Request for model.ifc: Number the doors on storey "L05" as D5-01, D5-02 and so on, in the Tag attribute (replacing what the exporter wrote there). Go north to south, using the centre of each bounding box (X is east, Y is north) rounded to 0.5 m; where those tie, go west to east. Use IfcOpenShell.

First a look at what the model holds.

```python
import ifcopenshell
import ifcopenshell.util.element
import ifcopenshell.util.placement

model = ifcopenshell.open("model.ifc")
print(model.schema)
storey = next(s for s in model.by_type("IfcBuildingStorey") if s.Name == "L05")
doors = [e for e in ifcopenshell.util.element.get_decomposition(storey) if e.is_a("IfcDoor")]
for e in sorted(doors, key=lambda e: e.id()):
    origin = ifcopenshell.util.placement.get_local_placement(e.ObjectPlacement)[:3, 3]
    print(e.id(), e.Tag, e.Name, origin.round(2) + 0.0, sep=" | ")
```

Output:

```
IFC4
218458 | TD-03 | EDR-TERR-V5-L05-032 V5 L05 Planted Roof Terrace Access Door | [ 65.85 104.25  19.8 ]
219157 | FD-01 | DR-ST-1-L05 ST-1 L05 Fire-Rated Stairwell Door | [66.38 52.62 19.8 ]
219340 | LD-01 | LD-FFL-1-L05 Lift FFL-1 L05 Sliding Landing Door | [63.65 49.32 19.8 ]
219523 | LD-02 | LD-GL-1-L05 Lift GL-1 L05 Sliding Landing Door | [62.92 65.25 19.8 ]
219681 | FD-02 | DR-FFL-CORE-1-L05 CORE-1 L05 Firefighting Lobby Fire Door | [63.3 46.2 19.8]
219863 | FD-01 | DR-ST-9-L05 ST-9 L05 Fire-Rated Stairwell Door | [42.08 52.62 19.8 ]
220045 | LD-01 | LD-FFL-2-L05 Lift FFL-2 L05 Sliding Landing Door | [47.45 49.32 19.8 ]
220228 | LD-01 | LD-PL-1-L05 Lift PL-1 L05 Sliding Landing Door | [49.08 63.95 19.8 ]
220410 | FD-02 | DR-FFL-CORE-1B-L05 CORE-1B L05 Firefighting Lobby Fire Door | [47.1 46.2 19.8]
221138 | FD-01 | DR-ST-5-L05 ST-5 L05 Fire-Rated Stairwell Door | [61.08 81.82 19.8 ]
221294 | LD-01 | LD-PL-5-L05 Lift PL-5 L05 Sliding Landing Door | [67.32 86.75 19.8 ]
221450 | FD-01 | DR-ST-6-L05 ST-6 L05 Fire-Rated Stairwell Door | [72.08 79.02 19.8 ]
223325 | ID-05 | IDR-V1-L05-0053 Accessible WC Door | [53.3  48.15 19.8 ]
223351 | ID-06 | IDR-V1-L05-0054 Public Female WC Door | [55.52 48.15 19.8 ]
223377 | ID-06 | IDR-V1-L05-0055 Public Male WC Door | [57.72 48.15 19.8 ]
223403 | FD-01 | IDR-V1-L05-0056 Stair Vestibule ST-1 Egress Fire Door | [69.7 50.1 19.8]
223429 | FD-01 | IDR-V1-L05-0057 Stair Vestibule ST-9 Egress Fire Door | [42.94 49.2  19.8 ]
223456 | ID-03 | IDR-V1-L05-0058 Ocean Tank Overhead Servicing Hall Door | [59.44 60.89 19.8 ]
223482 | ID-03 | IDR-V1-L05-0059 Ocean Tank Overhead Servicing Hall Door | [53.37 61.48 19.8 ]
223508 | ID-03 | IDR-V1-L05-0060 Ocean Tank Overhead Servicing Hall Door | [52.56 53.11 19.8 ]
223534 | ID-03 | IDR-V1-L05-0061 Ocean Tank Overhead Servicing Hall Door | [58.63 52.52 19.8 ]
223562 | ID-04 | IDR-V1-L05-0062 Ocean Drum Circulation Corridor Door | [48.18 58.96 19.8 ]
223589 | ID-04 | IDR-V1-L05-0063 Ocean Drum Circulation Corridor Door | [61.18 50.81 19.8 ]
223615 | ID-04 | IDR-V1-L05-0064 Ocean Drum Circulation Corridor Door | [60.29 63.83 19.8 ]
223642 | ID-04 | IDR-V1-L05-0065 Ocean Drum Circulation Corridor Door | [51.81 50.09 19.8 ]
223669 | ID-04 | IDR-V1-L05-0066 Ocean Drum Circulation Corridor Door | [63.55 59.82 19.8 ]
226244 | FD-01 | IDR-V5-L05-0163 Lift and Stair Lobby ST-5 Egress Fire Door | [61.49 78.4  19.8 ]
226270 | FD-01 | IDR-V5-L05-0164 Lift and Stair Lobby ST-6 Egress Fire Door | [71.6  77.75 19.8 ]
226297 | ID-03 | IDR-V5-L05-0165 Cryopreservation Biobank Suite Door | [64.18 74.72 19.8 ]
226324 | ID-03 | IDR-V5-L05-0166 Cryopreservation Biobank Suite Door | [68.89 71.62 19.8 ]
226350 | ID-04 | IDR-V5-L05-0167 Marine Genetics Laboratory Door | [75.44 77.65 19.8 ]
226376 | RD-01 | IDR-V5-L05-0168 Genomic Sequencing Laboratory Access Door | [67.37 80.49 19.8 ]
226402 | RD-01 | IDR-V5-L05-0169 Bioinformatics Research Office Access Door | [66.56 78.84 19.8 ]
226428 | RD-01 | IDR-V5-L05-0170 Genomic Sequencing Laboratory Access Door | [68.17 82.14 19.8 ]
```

```python
import ifcopenshell
import ifcopenshell.geom
import ifcopenshell.util.element
import ifcopenshell.util.shape

model = ifcopenshell.open("model.ifc")
settings = ifcopenshell.geom.settings()
settings.set("use-world-coords", True)


def centre(element):
    shape = ifcopenshell.geom.create_shape(settings, element)
    return ifcopenshell.util.shape.get_bbox_centroid(shape.geometry)


storey = next(s for s in model.by_type("IfcBuildingStorey") if s.Name == "L05")
doors = [e for e in ifcopenshell.util.element.get_decomposition(storey) if e.is_a("IfcDoor")]

# Insertion points can sit at a corner or the storey origin, so sort by the geometry (in metres).
centres = {e: centre(e) for e in doors}
doors.sort(key=lambda e: (-round(centres[e][1] / 0.5), centres[e][0]))

for i, e in enumerate(doors, start=1):
    number = f"D5-{i:02d}"
    e.Tag = number
    print(e.id(), number)

model.write("model_edited.ifc")
```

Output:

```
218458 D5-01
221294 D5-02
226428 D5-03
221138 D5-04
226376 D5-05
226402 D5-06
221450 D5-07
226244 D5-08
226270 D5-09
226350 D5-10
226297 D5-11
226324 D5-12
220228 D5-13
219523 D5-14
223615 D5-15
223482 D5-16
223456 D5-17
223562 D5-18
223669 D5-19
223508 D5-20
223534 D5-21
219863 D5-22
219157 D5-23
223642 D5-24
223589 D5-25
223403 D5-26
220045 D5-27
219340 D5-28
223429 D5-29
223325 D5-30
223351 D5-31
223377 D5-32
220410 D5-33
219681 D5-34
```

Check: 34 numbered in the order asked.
